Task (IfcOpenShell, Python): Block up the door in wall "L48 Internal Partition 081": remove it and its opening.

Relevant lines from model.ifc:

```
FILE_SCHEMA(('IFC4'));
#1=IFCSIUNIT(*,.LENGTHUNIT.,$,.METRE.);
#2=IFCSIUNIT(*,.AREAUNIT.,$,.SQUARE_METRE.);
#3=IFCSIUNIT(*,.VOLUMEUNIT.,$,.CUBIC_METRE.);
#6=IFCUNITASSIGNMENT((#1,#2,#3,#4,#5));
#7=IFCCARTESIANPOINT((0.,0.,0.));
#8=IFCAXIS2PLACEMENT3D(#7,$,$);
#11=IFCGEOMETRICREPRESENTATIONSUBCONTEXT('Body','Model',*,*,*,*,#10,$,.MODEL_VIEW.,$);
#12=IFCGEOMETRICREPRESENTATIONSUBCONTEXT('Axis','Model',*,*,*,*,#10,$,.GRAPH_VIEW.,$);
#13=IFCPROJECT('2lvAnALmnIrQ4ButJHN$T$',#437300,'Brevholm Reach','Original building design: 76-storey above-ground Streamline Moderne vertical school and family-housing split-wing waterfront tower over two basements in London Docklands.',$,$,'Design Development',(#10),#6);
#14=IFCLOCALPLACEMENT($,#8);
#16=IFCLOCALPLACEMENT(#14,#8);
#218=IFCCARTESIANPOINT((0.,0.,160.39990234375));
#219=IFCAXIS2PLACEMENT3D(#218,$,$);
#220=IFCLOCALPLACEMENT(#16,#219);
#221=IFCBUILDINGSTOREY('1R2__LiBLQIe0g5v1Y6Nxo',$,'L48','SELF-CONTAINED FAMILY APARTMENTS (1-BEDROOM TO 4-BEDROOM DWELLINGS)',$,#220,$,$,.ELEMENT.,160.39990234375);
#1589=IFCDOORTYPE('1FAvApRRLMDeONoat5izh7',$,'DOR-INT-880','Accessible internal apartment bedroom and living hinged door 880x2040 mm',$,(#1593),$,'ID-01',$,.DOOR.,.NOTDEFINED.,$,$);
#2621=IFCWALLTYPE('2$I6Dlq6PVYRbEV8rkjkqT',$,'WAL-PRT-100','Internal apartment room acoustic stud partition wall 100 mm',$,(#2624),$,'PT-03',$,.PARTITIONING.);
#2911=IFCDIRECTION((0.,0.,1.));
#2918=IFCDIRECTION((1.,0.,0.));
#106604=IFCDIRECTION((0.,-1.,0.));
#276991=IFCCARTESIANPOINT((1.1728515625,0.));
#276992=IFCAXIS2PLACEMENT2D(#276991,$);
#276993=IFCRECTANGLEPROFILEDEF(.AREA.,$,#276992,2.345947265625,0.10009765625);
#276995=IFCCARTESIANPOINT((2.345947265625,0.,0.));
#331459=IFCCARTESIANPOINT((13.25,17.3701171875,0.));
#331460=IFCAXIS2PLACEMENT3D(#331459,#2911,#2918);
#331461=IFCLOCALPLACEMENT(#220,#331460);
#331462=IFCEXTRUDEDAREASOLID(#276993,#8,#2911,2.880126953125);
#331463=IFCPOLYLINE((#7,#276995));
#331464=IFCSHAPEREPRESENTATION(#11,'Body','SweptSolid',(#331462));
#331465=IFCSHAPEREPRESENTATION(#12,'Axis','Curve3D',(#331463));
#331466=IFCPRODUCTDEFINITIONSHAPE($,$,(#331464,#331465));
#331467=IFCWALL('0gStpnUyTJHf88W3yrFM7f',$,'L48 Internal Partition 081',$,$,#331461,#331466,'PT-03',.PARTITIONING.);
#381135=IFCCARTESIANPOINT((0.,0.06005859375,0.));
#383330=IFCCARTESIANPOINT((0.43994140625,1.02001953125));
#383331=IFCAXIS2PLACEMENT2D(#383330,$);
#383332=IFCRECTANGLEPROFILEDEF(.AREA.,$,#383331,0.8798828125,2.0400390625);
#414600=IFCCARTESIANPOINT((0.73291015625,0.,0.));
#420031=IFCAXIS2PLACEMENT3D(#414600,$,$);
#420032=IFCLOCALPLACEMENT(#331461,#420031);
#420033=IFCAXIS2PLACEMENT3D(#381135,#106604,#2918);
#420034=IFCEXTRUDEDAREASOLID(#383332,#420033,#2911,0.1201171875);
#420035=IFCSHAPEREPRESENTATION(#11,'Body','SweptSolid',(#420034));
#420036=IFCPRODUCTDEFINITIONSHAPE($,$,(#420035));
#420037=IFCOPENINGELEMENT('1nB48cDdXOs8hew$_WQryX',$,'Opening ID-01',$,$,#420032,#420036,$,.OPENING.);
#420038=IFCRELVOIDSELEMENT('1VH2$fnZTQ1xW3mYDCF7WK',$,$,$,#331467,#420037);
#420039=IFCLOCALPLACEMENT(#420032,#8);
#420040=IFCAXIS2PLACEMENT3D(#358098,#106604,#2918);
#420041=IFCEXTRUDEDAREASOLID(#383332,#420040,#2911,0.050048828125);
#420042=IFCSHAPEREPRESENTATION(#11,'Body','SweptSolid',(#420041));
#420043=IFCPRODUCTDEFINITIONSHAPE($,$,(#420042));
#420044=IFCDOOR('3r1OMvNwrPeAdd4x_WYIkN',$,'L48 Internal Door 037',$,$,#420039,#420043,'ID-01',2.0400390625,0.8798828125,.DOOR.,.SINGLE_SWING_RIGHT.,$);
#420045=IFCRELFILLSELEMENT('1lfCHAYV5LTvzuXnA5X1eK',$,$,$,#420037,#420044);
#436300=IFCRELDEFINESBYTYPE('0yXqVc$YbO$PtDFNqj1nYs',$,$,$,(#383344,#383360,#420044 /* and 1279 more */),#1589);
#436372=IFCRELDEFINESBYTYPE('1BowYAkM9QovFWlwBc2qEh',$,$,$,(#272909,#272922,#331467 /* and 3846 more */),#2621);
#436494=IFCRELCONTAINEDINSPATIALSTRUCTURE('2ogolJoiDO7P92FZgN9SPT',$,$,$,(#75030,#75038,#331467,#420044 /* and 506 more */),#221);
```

```python
import ifcopenshell
import ifcopenshell.api.feature
import ifcopenshell.api.root
import ifcopenshell.geom
import ifcopenshell.util.shape

model = ifcopenshell.open("model.ifc")
settings = ifcopenshell.geom.settings()


def volume(element):
    """Net volume in cubic metres, openings subtracted."""
    shape = ifcopenshell.geom.create_shape(settings, element)
    return ifcopenshell.util.shape.get_volume(shape.geometry)


door = model.by_guid("3r1OMvNwrPeAdd4x_WYIkN")
opening = door.FillsVoids[0].RelatingOpeningElement
wall = opening.VoidsElements[0].RelatingBuildingElement
before = volume(wall)

ifcopenshell.api.root.remove_product(model, product=door)
ifcopenshell.api.feature.remove_feature(model, feature=opening)

after = volume(wall)

print(f"wall volume {before:.3f} -> {after:.3f} m3")

model.write("model_edited.ifc")
```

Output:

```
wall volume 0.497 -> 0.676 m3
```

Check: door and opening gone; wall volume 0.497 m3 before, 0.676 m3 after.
